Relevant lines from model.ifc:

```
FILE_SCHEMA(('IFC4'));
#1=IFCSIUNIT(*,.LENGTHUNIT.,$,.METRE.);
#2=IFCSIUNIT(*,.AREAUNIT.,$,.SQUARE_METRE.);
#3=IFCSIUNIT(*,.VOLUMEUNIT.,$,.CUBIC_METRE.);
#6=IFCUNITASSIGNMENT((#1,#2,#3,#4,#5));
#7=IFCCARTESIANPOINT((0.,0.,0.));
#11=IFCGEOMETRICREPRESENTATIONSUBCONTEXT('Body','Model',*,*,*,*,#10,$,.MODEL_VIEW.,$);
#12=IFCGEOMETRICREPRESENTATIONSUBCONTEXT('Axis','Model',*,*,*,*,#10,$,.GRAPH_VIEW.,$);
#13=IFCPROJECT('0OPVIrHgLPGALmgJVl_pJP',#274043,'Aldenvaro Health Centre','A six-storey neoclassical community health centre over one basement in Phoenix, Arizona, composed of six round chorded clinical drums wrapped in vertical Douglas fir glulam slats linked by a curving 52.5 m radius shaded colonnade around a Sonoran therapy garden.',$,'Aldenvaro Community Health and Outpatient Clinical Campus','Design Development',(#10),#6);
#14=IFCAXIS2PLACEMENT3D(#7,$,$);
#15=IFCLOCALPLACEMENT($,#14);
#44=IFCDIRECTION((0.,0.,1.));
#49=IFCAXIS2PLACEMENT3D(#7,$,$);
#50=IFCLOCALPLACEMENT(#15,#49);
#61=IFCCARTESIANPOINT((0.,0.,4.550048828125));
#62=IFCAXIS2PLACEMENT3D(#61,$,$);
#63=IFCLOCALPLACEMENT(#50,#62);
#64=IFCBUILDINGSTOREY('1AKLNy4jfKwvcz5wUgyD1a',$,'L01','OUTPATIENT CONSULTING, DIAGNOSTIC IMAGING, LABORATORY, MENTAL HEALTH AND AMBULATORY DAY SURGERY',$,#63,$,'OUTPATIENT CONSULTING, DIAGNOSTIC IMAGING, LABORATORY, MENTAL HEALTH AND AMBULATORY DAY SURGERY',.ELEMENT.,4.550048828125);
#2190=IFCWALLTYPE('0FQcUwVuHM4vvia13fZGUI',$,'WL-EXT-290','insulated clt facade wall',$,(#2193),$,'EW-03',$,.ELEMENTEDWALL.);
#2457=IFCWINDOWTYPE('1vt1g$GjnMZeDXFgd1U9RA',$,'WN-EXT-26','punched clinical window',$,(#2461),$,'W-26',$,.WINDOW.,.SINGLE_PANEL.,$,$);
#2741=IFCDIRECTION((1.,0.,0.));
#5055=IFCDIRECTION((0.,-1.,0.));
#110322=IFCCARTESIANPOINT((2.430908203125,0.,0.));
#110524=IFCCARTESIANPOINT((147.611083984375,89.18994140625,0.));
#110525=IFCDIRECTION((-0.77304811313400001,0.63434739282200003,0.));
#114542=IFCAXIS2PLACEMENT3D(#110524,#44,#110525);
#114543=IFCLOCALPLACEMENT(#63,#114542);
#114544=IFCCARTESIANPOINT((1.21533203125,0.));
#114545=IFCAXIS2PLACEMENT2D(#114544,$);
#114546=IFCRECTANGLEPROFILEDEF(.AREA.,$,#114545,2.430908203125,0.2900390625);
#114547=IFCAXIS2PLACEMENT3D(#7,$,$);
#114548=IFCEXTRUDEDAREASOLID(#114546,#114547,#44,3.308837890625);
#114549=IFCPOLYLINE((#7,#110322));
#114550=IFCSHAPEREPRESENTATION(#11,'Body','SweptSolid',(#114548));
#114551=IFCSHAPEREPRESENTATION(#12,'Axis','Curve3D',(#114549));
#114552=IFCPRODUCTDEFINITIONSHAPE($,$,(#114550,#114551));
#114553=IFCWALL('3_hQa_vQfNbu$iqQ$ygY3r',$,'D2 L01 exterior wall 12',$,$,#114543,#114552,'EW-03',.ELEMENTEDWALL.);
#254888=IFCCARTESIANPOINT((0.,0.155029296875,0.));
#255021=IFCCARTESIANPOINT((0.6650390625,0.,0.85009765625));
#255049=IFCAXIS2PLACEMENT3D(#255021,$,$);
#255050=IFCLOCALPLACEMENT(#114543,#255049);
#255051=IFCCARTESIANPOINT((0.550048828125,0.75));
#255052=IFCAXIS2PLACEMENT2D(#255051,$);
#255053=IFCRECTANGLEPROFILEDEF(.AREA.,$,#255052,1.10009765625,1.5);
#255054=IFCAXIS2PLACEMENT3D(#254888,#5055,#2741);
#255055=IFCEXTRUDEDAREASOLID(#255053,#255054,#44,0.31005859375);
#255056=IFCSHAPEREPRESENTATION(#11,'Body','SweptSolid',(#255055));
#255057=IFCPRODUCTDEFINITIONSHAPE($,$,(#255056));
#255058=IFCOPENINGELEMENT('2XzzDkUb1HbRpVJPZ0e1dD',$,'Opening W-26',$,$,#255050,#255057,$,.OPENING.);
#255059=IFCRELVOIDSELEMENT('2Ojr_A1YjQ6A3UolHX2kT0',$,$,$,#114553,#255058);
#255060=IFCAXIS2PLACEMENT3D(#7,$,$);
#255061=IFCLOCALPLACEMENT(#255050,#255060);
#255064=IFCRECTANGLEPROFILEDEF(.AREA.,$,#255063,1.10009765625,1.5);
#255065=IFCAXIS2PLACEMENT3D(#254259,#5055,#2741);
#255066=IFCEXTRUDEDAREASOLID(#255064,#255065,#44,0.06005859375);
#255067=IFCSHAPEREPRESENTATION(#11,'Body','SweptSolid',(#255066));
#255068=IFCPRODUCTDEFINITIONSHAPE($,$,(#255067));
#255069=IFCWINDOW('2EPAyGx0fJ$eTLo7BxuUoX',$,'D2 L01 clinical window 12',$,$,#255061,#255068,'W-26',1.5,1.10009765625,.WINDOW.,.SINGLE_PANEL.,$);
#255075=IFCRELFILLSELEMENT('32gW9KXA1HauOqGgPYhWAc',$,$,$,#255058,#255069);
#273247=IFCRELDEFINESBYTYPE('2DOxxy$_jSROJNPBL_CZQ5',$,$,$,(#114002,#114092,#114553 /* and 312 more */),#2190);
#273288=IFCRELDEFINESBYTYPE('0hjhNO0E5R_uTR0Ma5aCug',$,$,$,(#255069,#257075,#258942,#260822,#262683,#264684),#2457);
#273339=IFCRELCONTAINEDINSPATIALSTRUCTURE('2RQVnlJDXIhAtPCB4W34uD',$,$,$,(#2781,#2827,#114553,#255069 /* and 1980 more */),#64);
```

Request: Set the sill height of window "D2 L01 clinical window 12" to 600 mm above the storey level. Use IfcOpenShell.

```python
import numpy as np
import ifcopenshell
import ifcopenshell.api.geometry
import ifcopenshell.geom
import ifcopenshell.util.element
import ifcopenshell.util.placement
import ifcopenshell.util.shape
import ifcopenshell.util.unit

model = ifcopenshell.open("model.ifc")
unit_scale = ifcopenshell.util.unit.calculate_unit_scale(model)

window = model.by_guid("2EPAyGx0fJ$eTLo7BxuUoX")
opening = window.FillsVoids[0].RelatingOpeningElement
storey = ifcopenshell.util.element.get_container(window, ifc_class="IfcBuildingStorey")
level = ifcopenshell.util.placement.get_local_placement(storey.ObjectPlacement)[2, 3]

# The opening's origin need not be at the sill, so measure its lowest point.
shape = ifcopenshell.geom.create_shape(ifcopenshell.geom.settings(), opening)
bottom = ifcopenshell.util.shape.get_shape_bottom_elevation(shape, shape.geometry) / unit_scale
dz = level + 0.6 / unit_scale - bottom

shift = np.array([0.0, 0.0, dz])
# The window is placed relative to its opening, so it follows when the opening moves.
matrix = ifcopenshell.util.placement.get_local_placement(opening.ObjectPlacement)
matrix[:3, 3] += shift
ifcopenshell.api.geometry.edit_object_placement(
    model, product=opening, matrix=matrix, is_si=False, should_transform_children=True
)

print(f"moved by {dz * unit_scale:+.3f} m")

model.write("model-out.ifc")
```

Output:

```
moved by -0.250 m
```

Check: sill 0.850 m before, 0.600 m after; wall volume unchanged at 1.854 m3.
